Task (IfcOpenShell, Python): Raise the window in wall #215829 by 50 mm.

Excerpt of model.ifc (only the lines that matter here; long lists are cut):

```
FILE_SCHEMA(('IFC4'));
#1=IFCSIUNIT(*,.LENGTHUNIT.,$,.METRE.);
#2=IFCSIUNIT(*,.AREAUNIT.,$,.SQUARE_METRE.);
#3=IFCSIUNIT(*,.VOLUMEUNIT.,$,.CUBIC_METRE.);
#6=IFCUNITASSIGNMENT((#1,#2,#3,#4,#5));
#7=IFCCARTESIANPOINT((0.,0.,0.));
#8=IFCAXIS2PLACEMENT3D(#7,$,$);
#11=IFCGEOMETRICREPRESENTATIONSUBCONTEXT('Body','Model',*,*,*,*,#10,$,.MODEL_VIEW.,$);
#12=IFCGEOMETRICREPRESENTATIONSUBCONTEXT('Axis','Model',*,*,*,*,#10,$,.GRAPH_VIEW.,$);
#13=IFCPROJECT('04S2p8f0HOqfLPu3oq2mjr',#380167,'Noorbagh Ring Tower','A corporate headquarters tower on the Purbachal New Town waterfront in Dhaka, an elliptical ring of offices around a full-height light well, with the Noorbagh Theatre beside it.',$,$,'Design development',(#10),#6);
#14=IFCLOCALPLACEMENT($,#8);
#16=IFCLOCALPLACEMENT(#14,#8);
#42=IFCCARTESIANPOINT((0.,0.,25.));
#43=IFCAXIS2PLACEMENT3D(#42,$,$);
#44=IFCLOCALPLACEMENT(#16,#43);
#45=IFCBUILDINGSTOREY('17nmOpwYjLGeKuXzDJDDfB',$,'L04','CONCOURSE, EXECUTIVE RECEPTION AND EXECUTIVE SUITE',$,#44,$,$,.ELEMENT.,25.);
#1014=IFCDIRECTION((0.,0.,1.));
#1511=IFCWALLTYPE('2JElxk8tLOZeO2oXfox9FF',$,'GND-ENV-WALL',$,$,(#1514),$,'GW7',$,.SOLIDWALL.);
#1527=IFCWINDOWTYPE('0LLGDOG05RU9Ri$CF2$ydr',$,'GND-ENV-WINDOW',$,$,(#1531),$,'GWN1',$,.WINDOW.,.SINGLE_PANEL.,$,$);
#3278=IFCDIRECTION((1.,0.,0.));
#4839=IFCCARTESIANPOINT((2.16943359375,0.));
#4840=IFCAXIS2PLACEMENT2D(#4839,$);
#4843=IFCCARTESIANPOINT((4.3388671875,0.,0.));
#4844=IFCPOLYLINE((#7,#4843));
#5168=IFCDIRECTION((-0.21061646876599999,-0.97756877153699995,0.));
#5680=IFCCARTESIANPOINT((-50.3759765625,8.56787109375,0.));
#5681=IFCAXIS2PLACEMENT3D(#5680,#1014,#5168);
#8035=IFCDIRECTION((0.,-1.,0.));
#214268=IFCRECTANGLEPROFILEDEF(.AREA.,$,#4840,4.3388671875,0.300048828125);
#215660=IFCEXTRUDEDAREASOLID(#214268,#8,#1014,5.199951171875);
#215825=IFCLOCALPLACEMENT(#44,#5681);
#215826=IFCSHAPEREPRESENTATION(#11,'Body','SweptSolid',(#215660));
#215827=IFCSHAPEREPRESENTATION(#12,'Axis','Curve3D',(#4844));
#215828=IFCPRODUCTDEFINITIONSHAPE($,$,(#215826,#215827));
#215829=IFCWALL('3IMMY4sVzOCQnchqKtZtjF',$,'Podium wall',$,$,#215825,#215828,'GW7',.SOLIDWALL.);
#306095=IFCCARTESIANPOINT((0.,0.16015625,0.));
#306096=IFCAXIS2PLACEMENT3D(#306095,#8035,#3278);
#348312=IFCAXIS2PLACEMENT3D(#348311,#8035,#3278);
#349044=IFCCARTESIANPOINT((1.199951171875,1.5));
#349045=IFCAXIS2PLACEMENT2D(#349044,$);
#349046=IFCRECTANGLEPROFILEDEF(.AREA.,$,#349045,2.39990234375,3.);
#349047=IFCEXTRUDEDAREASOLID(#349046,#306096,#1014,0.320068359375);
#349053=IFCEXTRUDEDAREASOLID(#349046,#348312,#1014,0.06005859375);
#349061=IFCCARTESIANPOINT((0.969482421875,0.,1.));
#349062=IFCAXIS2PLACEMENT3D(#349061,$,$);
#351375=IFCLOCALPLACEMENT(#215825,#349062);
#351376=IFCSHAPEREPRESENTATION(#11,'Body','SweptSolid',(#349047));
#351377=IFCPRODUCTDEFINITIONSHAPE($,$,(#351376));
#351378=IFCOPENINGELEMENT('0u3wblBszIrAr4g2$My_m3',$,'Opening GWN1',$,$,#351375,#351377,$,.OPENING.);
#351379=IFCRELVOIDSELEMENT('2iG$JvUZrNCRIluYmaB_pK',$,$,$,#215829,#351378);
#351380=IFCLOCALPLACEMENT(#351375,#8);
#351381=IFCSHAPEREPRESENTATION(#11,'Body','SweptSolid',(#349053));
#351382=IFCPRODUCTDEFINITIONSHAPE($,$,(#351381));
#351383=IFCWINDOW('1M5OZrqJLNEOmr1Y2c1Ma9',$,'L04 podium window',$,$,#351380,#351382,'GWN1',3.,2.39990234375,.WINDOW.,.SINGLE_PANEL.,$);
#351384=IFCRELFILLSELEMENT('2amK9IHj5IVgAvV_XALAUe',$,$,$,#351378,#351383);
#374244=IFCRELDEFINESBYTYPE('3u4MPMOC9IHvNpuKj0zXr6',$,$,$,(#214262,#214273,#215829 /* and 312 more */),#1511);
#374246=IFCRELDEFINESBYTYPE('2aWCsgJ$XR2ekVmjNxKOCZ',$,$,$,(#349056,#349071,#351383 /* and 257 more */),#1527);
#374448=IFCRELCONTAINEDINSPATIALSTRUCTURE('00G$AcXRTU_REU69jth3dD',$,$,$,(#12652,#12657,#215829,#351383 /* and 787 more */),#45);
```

```python
import numpy as np
import ifcopenshell
import ifcopenshell.api.geometry
import ifcopenshell.util.placement
import ifcopenshell.util.unit

model = ifcopenshell.open("model.ifc")
unit_scale = ifcopenshell.util.unit.calculate_unit_scale(model)

window = model.by_guid("1M5OZrqJLNEOmr1Y2c1Ma9")
opening = window.FillsVoids[0].RelatingOpeningElement
dz = 0.05

shift = np.array([0.0, 0.0, dz])
# The window is placed relative to its opening, so it follows when the opening moves.
matrix = ifcopenshell.util.placement.get_local_placement(opening.ObjectPlacement)
matrix[:3, 3] += shift
ifcopenshell.api.geometry.edit_object_placement(
    model, product=opening, matrix=matrix, is_si=False, should_transform_children=True
)

print(f"moved by {dz * unit_scale:+.3f} m")

model.write("model-out.ifc")
```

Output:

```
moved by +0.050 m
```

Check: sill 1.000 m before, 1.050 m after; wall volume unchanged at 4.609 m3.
